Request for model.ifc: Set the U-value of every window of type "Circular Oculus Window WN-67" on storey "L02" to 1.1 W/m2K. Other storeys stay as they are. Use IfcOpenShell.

First a look at what the model holds.

```python
import ifcopenshell
import ifcopenshell.util.element

model = ifcopenshell.open("model.ifc")
print(model.schema)
storey = next(s for s in model.by_type("IfcBuildingStorey") if s.Name == "L02")
windows = [e for e in ifcopenshell.util.element.get_decomposition(storey) if e.is_a("IfcWindow")]
seen = {}
for e in windows:
    element_type = ifcopenshell.util.element.get_type(e)
    key = (element_type.Name if element_type != e and element_type else None, ifcopenshell.util.element.get_pset(e, "Pset_WindowCommon", "ThermalTransmittance"))
    seen[key] = seen.get(key, 0) + 1
for (name, value), count in sorted(seen.items(), key=str):
    print(count, "x", name, "|", value)
```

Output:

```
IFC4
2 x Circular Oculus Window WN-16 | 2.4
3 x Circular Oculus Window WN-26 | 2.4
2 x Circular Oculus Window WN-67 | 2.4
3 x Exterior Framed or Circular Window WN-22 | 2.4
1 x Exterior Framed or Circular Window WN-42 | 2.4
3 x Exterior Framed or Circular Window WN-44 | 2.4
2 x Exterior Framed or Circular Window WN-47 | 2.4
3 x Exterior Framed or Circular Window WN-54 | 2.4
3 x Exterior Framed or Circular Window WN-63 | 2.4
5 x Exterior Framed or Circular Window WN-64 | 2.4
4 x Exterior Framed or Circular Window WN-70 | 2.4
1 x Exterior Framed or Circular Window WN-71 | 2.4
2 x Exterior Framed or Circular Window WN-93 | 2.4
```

```python
import ifcopenshell
import ifcopenshell.api.pset
import ifcopenshell.util.element

model = ifcopenshell.open("model.ifc")

storey = next(s for s in model.by_type("IfcBuildingStorey") if s.Name == "L02")
windows = [e for e in ifcopenshell.util.element.get_decomposition(storey) if e.is_a("IfcWindow")]

count = 0
for e in windows:
    element_type = ifcopenshell.util.element.get_type(e)
    if element_type in (None, e) or element_type.Name != "Circular Oculus Window WN-67":
        continue
    # add_pset returns the element's existing set when there is one.
    pset = ifcopenshell.api.pset.add_pset(model, product=e, name="Pset_WindowCommon")
    ifcopenshell.api.pset.edit_pset(model, pset=pset, properties={"ThermalTransmittance": 1.1})
    count += 1

print(count, "windows updated")

model.write("model_rev.ifc")
```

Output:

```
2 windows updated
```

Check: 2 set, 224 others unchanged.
